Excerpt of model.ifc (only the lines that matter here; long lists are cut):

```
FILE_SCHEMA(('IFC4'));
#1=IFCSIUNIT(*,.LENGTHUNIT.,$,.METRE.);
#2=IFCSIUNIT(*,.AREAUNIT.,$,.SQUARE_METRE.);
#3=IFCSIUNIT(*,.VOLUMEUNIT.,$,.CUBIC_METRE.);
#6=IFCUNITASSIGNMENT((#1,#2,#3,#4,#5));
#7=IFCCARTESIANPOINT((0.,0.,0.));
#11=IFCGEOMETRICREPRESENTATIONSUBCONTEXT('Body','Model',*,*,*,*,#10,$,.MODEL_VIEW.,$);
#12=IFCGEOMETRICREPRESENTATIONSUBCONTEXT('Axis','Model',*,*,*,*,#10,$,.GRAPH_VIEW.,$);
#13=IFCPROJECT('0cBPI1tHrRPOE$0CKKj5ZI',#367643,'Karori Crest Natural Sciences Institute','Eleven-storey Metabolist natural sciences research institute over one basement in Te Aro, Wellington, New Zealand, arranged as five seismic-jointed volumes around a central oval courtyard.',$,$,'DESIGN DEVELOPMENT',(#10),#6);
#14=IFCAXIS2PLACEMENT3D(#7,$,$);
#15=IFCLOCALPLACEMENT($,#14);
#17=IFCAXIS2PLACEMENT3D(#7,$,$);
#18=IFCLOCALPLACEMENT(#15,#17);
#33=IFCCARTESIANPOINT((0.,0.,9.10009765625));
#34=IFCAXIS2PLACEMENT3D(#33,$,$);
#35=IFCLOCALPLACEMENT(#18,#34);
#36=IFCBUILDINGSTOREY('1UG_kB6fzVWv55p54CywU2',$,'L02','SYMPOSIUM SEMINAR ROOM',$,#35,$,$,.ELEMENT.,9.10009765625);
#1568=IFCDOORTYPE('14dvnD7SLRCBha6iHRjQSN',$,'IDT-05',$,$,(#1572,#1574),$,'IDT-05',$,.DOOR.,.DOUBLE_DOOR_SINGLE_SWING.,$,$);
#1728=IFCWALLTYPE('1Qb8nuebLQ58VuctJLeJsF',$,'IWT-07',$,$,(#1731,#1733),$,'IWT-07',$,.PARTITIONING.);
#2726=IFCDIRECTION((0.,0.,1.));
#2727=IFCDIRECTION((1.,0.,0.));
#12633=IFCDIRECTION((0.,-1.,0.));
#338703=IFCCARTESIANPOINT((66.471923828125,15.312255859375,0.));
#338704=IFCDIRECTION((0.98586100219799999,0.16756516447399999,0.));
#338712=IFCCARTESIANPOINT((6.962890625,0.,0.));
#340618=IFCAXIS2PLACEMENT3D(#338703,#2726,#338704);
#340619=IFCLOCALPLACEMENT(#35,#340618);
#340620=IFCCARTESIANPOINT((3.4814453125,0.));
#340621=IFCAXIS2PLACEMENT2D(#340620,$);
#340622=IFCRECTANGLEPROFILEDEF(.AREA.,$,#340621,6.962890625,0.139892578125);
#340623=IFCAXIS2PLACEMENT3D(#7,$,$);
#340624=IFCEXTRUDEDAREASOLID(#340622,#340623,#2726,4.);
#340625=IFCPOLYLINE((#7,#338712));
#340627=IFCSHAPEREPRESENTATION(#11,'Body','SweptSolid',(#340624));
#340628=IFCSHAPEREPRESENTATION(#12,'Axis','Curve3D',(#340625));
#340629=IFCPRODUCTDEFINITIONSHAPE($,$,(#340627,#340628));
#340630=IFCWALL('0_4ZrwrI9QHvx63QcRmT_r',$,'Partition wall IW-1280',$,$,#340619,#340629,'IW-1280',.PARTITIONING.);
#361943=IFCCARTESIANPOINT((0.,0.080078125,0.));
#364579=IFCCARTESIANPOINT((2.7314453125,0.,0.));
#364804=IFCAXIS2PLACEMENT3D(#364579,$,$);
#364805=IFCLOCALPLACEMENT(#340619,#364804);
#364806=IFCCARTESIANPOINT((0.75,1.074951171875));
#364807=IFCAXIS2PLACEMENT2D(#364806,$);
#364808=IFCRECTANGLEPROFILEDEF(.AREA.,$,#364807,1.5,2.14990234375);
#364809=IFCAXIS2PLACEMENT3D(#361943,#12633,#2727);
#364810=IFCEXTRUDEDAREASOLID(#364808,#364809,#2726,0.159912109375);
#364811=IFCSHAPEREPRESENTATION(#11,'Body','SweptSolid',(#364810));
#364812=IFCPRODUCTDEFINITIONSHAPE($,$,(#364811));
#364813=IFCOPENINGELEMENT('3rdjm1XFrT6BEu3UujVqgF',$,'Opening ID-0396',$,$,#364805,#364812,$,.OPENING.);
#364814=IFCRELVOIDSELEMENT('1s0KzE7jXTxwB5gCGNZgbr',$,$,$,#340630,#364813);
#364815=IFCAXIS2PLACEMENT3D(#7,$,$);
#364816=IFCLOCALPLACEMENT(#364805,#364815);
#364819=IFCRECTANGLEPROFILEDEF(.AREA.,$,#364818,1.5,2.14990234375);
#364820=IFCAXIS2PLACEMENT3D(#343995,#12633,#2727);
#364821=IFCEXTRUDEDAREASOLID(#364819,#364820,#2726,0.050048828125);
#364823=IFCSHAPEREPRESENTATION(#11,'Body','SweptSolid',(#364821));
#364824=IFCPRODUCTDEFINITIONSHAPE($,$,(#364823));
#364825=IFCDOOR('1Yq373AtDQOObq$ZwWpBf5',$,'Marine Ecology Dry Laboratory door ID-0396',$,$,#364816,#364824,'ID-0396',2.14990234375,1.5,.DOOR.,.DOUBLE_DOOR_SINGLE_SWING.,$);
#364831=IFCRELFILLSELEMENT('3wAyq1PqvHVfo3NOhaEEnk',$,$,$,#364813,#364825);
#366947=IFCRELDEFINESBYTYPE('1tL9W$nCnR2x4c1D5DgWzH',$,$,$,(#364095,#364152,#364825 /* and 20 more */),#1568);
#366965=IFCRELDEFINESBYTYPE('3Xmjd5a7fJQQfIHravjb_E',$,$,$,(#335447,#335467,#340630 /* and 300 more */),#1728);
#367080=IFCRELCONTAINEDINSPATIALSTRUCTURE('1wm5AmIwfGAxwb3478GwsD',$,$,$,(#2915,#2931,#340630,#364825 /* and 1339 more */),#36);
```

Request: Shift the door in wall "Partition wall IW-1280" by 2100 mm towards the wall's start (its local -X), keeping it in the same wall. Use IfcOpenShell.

```python
import ifcopenshell
import ifcopenshell.api.geometry
import ifcopenshell.util.placement
import ifcopenshell.util.unit

model = ifcopenshell.open("model.ifc")
unit_scale = ifcopenshell.util.unit.calculate_unit_scale(model)

door = model.by_guid("1Yq373AtDQOObq$ZwWpBf5")
opening = door.FillsVoids[0].RelatingOpeningElement
wall = opening.VoidsElements[0].RelatingBuildingElement

wall_matrix = ifcopenshell.util.placement.get_local_placement(wall.ObjectPlacement)
shift = wall_matrix[:3, 0] * -2.1 / unit_scale
before = ifcopenshell.util.placement.get_local_placement(door.ObjectPlacement)[:3, 3].copy()

# The door is placed relative to its opening, so it follows when the opening moves.
matrix = ifcopenshell.util.placement.get_local_placement(opening.ObjectPlacement)
matrix[:3, 3] += shift
ifcopenshell.api.geometry.edit_object_placement(
    model, product=opening, matrix=matrix, is_si=False, should_transform_children=True
)

after = ifcopenshell.util.placement.get_local_placement(door.ObjectPlacement)[:3, 3]
print("door moved by", (after - before).round(3) + 0.0)

model.write("model-out.ifc")
```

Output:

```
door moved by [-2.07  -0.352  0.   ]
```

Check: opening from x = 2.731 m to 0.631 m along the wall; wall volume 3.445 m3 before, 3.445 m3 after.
